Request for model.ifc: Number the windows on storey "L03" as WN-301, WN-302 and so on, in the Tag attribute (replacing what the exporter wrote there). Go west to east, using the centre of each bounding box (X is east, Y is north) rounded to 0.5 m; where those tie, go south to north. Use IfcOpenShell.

First a look at what the model holds.

```python
import ifcopenshell
import ifcopenshell.util.element
import ifcopenshell.util.placement

model = ifcopenshell.open("model.ifc")
print(model.schema)
storey = next(s for s in model.by_type("IfcBuildingStorey") if s.Name == "L03")
windows = [e for e in ifcopenshell.util.element.get_decomposition(storey) if e.is_a("IfcWindow")]
for e in sorted(windows, key=lambda e: e.id()):
    origin = ifcopenshell.util.placement.get_local_placement(e.ObjectPlacement)[:3, 3]
    print(e.id(), e.Tag, e.Name, origin.round(2) + 0.0, sep=" | ")
```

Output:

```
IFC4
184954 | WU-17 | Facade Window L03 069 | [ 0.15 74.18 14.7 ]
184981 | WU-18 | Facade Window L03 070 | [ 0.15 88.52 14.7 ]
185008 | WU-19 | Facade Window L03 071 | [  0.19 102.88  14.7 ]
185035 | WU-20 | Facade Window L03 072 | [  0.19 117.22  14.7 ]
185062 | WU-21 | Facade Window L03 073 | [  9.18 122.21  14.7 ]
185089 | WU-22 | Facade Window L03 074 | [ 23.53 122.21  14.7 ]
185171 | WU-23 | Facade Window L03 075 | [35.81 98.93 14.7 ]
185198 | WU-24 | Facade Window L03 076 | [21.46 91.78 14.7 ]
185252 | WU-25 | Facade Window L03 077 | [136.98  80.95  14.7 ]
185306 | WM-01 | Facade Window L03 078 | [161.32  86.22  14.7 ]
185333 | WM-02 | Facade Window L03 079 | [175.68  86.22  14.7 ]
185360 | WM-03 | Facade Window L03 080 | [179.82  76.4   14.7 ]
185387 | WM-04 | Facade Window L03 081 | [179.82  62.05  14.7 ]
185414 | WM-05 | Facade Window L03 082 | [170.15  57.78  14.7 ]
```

```python
import ifcopenshell
import ifcopenshell.geom
import ifcopenshell.util.element
import ifcopenshell.util.shape

model = ifcopenshell.open("model.ifc")
settings = ifcopenshell.geom.settings()
settings.set("use-world-coords", True)


def centre(element):
    shape = ifcopenshell.geom.create_shape(settings, element)
    return ifcopenshell.util.shape.get_bbox_centroid(shape.geometry)


storey = next(s for s in model.by_type("IfcBuildingStorey") if s.Name == "L03")
windows = [e for e in ifcopenshell.util.element.get_decomposition(storey) if e.is_a("IfcWindow")]

# Insertion points can sit at a corner or the storey origin, so sort by the geometry (in metres).
centres = {e: centre(e) for e in windows}
windows.sort(key=lambda e: (round(centres[e][0] / 0.5), centres[e][1]))

for i, e in enumerate(windows, start=1):
    number = f"WN-3{i:02d}"
    e.Tag = number
    print(e.id(), number)

model.write("model_updated.ifc")
```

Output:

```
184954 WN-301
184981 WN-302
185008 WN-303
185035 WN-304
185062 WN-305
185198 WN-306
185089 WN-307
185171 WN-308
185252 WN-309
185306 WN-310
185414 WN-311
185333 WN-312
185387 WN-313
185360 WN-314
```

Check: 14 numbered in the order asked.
